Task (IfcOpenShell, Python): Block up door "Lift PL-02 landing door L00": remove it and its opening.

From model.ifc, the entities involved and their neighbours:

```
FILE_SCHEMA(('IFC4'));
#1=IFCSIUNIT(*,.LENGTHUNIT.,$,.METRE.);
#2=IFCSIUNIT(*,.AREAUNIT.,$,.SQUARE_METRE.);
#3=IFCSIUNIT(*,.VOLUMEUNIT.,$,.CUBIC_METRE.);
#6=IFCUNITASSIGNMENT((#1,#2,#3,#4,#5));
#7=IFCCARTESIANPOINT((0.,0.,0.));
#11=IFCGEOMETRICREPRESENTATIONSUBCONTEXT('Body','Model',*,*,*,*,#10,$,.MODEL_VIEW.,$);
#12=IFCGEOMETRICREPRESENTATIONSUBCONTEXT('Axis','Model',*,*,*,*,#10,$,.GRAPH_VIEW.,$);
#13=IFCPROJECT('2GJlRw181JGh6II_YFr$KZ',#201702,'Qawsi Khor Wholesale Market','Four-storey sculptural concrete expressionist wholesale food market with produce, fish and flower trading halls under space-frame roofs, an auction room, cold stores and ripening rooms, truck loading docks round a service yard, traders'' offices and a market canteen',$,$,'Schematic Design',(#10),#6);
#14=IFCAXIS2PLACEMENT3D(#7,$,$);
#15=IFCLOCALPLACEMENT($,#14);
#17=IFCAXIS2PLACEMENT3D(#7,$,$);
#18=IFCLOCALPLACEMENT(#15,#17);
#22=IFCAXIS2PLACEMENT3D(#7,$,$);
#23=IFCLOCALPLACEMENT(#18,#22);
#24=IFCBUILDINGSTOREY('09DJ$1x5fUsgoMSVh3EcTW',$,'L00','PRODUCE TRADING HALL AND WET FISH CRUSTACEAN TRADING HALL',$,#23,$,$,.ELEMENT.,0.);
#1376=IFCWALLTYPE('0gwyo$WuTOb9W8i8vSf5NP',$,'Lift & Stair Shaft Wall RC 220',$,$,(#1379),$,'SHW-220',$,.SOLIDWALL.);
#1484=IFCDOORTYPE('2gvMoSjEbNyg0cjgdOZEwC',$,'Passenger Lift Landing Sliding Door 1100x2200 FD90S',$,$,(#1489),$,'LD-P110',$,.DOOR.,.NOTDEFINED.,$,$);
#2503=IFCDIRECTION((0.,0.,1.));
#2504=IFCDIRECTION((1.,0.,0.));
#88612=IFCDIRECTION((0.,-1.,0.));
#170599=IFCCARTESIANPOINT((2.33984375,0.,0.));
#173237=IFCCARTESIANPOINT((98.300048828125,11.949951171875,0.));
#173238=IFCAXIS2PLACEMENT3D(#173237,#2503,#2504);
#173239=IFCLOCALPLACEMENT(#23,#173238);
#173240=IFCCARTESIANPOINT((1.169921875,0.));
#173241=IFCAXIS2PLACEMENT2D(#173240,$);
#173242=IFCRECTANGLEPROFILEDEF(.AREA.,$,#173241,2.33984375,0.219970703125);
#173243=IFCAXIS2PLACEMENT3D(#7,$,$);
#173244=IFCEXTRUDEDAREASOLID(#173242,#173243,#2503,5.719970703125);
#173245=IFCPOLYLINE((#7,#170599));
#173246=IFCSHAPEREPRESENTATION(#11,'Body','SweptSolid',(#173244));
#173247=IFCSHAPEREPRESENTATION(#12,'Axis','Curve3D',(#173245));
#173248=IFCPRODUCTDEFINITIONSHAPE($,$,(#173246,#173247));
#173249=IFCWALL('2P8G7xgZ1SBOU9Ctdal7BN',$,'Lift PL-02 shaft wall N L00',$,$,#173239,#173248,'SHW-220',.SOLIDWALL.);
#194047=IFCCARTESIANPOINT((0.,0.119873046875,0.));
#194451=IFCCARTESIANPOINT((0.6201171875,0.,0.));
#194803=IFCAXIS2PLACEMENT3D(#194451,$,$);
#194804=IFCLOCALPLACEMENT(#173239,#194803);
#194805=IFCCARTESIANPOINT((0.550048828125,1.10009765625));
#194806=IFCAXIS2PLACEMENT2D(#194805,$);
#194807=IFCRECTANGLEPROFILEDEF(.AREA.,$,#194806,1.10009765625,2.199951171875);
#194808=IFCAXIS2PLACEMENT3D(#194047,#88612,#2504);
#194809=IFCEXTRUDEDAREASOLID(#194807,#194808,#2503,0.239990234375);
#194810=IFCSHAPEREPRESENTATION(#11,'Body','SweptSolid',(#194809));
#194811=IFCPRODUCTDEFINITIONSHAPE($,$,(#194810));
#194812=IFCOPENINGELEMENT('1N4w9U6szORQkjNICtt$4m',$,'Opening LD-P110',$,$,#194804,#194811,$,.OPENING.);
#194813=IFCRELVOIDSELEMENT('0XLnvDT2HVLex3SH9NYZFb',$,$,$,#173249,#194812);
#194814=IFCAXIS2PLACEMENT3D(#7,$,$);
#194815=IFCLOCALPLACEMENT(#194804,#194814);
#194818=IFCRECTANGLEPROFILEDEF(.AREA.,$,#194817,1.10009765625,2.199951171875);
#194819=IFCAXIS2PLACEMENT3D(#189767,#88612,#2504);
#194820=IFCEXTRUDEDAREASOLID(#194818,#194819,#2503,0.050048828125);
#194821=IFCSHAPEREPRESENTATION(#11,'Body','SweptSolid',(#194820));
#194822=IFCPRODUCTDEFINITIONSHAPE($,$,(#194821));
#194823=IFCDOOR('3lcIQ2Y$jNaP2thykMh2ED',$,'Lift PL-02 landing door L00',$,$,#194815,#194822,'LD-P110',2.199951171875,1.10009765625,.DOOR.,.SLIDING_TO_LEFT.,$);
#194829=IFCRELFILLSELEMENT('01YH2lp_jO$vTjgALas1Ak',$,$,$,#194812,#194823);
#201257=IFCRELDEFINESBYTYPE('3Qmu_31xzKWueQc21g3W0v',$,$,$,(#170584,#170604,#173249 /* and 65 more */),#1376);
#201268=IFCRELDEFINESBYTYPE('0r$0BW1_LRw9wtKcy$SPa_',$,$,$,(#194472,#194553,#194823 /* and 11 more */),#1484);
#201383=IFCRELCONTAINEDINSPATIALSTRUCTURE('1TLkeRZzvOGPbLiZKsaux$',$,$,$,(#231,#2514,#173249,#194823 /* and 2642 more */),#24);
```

```python
import ifcopenshell
import ifcopenshell.api.feature
import ifcopenshell.api.root
import ifcopenshell.geom
import ifcopenshell.util.shape

model = ifcopenshell.open("model.ifc")
settings = ifcopenshell.geom.settings()


def volume(element):
    """Net volume in cubic metres, openings subtracted."""
    shape = ifcopenshell.geom.create_shape(settings, element)
    return ifcopenshell.util.shape.get_volume(shape.geometry)


door = model.by_guid("3lcIQ2Y$jNaP2thykMh2ED")
opening = door.FillsVoids[0].RelatingOpeningElement
wall = opening.VoidsElements[0].RelatingBuildingElement
before = volume(wall)

ifcopenshell.api.root.remove_product(model, product=door)
ifcopenshell.api.feature.remove_feature(model, feature=opening)

after = volume(wall)

print(f"wall volume {before:.3f} -> {after:.3f} m3")

model.write("model_rev.ifc")
```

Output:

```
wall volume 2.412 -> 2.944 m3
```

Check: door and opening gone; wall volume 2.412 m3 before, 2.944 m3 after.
